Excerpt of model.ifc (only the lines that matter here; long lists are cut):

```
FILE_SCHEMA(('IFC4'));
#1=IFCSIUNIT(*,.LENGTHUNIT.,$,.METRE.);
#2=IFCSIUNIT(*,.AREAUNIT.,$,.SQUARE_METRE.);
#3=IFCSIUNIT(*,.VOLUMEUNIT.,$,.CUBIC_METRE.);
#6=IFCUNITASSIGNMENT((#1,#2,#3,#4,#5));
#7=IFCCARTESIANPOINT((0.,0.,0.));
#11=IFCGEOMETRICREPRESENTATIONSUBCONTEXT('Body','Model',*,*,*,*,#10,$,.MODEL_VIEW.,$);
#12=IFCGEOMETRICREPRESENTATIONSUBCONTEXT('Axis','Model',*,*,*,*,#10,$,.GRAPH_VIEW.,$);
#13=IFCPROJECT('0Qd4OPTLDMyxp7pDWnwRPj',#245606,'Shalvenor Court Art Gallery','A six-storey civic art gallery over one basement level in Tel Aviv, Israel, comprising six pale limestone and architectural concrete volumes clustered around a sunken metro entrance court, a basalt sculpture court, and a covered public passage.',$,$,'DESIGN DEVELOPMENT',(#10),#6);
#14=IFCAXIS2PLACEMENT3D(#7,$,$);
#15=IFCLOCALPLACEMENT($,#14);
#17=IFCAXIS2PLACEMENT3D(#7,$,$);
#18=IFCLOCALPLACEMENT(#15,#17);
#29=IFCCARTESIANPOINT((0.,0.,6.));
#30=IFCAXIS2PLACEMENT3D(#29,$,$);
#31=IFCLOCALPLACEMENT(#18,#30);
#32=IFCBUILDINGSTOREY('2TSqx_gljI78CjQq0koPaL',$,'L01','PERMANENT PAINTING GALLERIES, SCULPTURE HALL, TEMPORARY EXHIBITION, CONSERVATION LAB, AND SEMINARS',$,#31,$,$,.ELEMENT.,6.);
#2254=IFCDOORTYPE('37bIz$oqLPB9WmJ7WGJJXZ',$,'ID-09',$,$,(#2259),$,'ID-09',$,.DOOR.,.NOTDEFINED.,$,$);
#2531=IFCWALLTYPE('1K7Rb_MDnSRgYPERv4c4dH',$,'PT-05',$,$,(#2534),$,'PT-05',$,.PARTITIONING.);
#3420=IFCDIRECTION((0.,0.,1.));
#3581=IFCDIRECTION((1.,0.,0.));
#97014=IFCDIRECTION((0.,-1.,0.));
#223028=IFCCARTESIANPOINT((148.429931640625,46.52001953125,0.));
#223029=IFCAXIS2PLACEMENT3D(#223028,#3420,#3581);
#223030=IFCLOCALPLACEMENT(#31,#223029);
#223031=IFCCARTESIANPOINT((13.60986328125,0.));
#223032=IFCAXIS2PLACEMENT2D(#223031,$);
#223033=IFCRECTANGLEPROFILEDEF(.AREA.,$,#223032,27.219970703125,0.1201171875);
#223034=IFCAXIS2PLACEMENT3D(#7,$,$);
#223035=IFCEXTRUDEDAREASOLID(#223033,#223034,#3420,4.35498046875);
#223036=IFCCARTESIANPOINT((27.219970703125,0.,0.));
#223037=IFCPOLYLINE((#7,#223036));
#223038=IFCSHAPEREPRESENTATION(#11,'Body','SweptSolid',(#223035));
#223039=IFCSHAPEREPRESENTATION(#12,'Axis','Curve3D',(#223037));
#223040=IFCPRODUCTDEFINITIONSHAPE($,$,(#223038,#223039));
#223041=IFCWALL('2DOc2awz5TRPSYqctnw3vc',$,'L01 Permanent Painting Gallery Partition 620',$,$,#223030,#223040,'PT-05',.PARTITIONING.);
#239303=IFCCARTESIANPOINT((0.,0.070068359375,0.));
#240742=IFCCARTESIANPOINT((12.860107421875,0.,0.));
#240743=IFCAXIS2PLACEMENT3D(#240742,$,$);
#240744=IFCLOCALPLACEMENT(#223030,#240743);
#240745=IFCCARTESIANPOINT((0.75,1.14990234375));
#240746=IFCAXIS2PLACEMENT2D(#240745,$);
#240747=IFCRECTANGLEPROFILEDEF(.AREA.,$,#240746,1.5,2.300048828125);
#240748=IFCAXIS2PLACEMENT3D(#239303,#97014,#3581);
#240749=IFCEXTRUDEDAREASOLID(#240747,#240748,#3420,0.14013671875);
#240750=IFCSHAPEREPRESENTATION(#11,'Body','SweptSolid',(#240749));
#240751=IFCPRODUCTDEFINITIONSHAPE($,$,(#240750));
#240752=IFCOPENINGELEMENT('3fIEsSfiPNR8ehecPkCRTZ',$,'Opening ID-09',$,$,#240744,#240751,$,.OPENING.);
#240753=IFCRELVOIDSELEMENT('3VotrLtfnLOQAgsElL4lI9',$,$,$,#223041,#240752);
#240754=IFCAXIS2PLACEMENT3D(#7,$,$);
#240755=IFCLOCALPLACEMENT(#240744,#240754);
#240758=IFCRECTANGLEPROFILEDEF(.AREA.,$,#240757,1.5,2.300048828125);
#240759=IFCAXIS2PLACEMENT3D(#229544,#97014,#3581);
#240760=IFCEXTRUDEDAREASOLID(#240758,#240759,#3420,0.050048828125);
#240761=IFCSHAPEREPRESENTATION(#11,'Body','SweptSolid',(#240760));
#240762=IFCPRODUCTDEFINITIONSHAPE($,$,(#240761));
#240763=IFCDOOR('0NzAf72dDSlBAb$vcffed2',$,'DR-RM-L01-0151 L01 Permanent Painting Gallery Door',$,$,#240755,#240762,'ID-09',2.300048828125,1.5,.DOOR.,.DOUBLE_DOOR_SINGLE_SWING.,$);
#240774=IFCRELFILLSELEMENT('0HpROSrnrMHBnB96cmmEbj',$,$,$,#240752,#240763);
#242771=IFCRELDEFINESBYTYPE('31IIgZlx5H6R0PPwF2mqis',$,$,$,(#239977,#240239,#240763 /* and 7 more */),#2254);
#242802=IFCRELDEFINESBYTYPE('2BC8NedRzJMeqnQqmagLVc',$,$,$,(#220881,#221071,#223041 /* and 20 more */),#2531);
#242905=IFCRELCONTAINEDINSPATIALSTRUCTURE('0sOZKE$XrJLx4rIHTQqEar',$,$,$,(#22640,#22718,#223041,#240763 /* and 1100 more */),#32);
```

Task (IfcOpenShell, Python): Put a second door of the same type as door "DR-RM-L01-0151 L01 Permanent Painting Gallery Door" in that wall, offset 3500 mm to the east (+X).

```python
import ifcopenshell
import ifcopenshell.api.feature
import ifcopenshell.api.geometry
import ifcopenshell.api.root
import ifcopenshell.geom
import ifcopenshell.util.element
import ifcopenshell.util.placement
import ifcopenshell.util.shape

model = ifcopenshell.open("model.ifc")
settings = ifcopenshell.geom.settings()


def volume(element):
    """Net volume in cubic metres, openings subtracted."""
    shape = ifcopenshell.geom.create_shape(settings, element)
    return ifcopenshell.util.shape.get_volume(shape.geometry)


door = model.by_guid("0NzAf72dDSlBAb$vcffed2")
opening = door.FillsVoids[0].RelatingOpeningElement
wall = opening.VoidsElements[0].RelatingBuildingElement
before = volume(wall)
shift = ifcopenshell.util.placement.get_local_placement(wall.ObjectPlacement)[:3, 0] * 3.5

# copy_class copies the void relationship, type, container and properties, but no geometry.
new_opening = ifcopenshell.api.root.copy_class(model, product=opening)
new_opening.Representation = ifcopenshell.util.element.copy_deep(
    model, opening.Representation, exclude=["IfcGeometricRepresentationContext", "IfcRepresentationMap"]
)
new_door = ifcopenshell.api.root.copy_class(model, product=door)
new_door.Representation = ifcopenshell.util.element.copy_deep(
    model, door.Representation, exclude=["IfcGeometricRepresentationContext", "IfcRepresentationMap"]
)
new_door.Tag = None
ifcopenshell.api.feature.add_filling(model, opening=new_opening, element=new_door)

for old, new in ((opening, new_opening), (door, new_door)):
    matrix = ifcopenshell.util.placement.get_local_placement(old.ObjectPlacement)
    matrix[:3, 3] += shift
    ifcopenshell.api.geometry.edit_object_placement(model, product=new, matrix=matrix, is_si=False)

after = volume(wall)

print(f"wall volume {before:.3f} -> {after:.3f} m3")

model.write("model_edited.ifc")
```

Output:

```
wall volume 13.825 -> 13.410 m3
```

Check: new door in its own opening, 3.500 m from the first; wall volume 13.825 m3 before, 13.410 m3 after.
